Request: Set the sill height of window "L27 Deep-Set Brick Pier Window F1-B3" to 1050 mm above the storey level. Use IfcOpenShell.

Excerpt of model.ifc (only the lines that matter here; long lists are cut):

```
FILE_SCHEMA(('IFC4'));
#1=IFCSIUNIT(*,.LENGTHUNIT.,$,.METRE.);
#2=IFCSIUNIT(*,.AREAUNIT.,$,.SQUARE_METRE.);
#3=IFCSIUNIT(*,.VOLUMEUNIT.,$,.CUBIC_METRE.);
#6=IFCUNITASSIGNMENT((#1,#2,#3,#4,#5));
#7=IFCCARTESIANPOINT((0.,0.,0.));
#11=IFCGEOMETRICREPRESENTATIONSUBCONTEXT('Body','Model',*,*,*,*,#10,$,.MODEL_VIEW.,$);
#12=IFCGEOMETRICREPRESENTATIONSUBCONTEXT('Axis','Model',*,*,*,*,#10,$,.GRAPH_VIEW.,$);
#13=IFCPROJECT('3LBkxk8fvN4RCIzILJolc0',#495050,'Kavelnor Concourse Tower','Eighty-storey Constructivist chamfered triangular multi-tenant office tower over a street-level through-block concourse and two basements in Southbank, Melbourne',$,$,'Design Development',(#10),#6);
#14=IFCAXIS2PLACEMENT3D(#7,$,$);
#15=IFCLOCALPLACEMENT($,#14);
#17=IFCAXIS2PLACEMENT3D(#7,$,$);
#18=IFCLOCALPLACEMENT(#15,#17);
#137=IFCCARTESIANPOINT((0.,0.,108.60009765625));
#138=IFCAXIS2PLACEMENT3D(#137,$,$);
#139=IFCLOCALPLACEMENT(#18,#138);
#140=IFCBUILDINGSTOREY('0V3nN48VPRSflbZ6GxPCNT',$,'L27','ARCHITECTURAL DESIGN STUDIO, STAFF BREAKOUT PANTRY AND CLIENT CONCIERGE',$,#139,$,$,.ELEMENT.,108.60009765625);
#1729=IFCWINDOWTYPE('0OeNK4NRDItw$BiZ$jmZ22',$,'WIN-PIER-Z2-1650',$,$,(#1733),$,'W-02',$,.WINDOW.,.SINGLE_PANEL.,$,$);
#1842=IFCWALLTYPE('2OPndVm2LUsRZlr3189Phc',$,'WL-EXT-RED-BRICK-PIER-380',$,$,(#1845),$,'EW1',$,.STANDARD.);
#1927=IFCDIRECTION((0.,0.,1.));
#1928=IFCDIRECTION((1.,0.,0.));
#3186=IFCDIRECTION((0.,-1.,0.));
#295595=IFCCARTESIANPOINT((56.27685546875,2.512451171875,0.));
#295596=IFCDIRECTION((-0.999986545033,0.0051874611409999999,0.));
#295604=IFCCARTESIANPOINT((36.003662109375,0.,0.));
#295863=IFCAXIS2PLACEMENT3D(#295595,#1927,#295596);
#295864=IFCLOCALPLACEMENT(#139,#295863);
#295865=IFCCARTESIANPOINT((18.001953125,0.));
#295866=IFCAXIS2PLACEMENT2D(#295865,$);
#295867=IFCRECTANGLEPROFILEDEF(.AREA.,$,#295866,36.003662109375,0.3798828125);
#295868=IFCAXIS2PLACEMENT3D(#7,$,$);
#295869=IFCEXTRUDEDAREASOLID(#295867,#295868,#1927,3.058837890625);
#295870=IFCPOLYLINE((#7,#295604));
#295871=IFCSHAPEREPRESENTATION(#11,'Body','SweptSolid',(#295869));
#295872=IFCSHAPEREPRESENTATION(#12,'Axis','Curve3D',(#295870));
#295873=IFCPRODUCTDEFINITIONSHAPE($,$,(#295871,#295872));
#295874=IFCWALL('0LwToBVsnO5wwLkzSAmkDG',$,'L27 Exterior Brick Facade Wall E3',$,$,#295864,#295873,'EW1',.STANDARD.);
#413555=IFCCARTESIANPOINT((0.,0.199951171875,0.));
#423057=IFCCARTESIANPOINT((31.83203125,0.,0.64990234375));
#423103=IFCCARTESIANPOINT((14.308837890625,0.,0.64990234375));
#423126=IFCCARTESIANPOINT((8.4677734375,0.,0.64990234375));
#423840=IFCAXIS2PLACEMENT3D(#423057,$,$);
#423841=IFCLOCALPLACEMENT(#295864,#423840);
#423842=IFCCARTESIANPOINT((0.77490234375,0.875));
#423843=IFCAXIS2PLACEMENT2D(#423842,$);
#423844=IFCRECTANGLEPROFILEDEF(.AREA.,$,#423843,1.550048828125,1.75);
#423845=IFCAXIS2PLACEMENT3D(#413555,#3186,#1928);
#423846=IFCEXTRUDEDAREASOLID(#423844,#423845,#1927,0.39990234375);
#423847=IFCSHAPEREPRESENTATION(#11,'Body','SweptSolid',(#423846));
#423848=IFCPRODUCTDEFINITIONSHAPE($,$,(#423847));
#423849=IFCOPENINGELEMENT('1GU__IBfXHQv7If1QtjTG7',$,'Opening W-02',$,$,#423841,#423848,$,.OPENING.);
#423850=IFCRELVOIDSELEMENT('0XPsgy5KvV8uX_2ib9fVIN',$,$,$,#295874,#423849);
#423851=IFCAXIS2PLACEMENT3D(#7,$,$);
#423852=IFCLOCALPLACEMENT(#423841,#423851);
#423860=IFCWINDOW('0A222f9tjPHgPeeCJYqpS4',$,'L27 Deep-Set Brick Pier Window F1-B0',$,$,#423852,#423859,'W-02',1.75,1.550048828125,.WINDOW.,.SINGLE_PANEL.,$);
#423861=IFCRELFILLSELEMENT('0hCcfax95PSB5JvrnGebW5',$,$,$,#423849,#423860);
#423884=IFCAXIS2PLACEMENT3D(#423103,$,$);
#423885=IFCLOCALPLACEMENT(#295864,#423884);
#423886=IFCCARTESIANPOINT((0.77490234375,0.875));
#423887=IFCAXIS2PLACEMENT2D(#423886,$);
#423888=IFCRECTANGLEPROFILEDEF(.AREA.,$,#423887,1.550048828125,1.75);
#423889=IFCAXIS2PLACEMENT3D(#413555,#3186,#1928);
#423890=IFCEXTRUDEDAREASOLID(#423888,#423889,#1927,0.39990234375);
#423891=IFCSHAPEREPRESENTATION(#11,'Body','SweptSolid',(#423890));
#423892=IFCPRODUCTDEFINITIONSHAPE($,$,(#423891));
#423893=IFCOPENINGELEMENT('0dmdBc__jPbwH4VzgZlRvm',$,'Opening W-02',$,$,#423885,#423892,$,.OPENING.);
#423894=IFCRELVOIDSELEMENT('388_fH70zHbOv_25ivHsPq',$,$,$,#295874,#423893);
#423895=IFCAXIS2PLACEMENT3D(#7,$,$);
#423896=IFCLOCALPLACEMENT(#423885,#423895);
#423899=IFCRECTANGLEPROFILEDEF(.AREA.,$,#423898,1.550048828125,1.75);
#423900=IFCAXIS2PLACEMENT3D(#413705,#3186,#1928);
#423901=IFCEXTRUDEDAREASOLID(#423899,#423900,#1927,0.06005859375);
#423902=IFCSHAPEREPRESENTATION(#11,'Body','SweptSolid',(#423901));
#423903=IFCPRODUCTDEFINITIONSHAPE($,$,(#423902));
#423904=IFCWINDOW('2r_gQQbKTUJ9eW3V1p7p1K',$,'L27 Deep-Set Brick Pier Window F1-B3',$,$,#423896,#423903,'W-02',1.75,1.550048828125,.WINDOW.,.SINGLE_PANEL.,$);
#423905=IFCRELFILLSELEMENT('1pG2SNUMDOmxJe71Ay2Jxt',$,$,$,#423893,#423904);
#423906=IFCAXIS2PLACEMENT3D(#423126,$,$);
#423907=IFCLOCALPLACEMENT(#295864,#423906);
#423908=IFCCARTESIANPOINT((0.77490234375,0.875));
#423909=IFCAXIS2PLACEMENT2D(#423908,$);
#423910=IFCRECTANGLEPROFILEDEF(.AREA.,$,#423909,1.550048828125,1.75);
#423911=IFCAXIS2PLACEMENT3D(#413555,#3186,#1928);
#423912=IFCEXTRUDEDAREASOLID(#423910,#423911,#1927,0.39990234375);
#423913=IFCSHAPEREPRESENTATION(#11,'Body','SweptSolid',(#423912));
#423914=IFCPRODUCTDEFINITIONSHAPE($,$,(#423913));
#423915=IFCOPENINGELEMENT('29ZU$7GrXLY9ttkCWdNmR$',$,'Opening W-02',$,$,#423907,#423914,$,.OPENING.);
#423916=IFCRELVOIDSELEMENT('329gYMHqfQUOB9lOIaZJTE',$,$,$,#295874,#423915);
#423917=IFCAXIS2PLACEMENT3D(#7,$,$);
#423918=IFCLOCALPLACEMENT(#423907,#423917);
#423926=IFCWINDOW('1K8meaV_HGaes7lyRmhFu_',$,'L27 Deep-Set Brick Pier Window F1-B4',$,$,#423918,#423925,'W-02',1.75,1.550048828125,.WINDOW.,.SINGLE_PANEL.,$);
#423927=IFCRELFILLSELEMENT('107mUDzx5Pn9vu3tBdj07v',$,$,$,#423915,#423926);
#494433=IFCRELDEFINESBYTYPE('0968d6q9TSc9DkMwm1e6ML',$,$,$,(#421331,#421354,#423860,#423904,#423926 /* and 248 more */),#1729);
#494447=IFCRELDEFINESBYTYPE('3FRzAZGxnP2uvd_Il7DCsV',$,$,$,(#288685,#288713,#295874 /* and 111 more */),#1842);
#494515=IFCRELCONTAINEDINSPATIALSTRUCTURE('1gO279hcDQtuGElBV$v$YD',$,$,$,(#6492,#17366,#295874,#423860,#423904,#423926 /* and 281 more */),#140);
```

```python
import numpy as np
import ifcopenshell
import ifcopenshell.api.geometry
import ifcopenshell.geom
import ifcopenshell.util.element
import ifcopenshell.util.placement
import ifcopenshell.util.shape
import ifcopenshell.util.unit

model = ifcopenshell.open("model.ifc")
unit_scale = ifcopenshell.util.unit.calculate_unit_scale(model)

window = model.by_id(423904)
opening = window.FillsVoids[0].RelatingOpeningElement
storey = ifcopenshell.util.element.get_container(window, ifc_class="IfcBuildingStorey")
level = ifcopenshell.util.placement.get_local_placement(storey.ObjectPlacement)[2, 3]

# The opening's origin need not be at the sill, so measure its lowest point.
shape = ifcopenshell.geom.create_shape(ifcopenshell.geom.settings(), opening)
bottom = ifcopenshell.util.shape.get_shape_bottom_elevation(shape, shape.geometry) / unit_scale
dz = level + 1.05 / unit_scale - bottom

shift = np.array([0.0, 0.0, dz])
# The window is placed relative to its opening, so it follows when the opening moves.
matrix = ifcopenshell.util.placement.get_local_placement(opening.ObjectPlacement)
matrix[:3, 3] += shift
ifcopenshell.api.geometry.edit_object_placement(
    model, product=opening, matrix=matrix, is_si=False, should_transform_children=True
)

print(f"moved by {dz * unit_scale:+.3f} m")

model.write("model_v2.ifc")
```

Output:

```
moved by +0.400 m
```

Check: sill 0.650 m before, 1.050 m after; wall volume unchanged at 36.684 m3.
